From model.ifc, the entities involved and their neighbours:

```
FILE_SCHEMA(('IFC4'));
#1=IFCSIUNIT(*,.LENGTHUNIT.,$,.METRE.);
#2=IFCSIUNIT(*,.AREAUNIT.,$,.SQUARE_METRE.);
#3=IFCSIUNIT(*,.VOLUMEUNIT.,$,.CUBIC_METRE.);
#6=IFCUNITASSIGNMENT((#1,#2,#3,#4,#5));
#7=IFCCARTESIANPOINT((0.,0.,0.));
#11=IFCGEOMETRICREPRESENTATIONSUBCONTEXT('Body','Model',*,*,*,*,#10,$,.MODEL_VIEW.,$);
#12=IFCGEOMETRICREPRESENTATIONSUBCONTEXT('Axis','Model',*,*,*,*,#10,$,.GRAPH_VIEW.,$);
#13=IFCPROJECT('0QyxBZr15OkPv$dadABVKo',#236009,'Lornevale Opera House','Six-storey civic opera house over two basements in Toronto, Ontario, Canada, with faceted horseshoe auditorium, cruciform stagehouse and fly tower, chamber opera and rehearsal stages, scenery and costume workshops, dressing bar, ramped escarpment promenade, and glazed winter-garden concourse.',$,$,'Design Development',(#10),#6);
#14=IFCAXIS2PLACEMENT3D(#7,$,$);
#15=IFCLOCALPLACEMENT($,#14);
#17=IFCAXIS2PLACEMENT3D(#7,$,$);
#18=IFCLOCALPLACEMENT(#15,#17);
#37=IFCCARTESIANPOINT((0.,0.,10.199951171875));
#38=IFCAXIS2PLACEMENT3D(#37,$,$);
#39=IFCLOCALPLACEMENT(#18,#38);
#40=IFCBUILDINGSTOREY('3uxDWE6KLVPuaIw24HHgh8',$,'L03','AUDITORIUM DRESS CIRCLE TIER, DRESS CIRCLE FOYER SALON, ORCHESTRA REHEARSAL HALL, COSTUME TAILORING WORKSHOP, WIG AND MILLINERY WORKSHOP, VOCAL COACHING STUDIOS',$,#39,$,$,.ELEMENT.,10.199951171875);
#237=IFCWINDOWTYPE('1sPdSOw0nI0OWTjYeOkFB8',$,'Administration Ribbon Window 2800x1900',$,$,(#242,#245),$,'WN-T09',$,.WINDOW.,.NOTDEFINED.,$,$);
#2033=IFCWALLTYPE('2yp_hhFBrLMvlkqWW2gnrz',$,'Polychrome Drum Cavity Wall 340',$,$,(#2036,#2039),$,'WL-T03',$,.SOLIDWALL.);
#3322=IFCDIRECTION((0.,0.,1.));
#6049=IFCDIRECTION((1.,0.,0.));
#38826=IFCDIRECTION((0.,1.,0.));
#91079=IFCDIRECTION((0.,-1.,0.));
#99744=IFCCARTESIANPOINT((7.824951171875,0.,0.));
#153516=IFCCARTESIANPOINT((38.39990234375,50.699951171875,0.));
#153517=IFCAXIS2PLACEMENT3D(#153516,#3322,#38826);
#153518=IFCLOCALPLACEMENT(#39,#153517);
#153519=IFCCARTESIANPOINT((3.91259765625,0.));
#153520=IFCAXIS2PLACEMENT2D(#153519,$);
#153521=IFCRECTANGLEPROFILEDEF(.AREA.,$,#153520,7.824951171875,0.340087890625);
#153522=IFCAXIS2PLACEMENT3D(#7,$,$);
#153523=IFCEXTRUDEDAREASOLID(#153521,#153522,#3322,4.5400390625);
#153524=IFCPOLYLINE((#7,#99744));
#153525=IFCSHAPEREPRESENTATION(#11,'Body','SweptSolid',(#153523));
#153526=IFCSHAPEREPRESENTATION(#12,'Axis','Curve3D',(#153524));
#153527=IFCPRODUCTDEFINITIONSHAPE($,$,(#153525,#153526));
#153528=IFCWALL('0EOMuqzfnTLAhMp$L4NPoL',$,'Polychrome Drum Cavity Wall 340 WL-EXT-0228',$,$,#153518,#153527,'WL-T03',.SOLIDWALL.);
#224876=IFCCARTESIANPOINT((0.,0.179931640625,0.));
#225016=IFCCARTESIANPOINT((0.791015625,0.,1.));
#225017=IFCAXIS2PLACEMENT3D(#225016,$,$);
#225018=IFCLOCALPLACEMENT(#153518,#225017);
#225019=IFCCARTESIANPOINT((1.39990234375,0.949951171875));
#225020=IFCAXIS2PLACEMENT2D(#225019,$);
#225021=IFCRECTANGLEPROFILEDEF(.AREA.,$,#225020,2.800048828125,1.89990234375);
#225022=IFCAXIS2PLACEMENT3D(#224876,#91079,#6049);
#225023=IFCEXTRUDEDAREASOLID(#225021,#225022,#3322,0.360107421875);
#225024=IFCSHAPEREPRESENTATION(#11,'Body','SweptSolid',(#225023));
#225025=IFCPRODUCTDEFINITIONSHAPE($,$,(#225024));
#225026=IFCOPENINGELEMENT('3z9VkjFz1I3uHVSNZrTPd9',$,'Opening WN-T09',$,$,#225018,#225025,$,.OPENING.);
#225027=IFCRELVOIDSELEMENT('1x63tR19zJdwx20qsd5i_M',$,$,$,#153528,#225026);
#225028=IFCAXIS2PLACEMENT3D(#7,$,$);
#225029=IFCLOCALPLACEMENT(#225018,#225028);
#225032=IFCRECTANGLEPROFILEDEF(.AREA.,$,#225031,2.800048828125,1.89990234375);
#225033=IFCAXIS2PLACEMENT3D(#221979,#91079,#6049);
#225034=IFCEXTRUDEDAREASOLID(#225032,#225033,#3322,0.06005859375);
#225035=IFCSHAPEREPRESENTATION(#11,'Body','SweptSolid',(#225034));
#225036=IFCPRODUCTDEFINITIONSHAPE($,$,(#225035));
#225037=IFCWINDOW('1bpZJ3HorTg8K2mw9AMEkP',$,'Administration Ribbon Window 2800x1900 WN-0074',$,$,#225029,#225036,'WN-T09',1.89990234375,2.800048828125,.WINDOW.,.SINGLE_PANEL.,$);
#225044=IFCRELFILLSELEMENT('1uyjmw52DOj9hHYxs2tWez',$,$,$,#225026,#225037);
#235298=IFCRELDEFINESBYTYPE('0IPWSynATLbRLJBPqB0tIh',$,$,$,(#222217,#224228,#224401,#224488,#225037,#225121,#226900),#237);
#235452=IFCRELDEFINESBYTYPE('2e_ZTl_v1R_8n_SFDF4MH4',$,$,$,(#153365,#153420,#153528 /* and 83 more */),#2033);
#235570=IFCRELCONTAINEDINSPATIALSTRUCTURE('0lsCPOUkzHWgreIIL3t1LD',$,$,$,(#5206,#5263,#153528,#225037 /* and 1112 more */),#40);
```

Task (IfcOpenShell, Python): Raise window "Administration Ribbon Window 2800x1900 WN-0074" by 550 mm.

```python
import numpy as np
import ifcopenshell
import ifcopenshell.api.geometry
import ifcopenshell.util.placement
import ifcopenshell.util.unit

model = ifcopenshell.open("model.ifc")
unit_scale = ifcopenshell.util.unit.calculate_unit_scale(model)

window = model.by_guid("1bpZJ3HorTg8K2mw9AMEkP")
opening = window.FillsVoids[0].RelatingOpeningElement
dz = 0.55

shift = np.array([0.0, 0.0, dz])
# The window is placed relative to its opening, so it follows when the opening moves.
matrix = ifcopenshell.util.placement.get_local_placement(opening.ObjectPlacement)
matrix[:3, 3] += shift
ifcopenshell.api.geometry.edit_object_placement(
    model, product=opening, matrix=matrix, is_si=False, should_transform_children=True
)

print(f"moved by {dz * unit_scale:+.3f} m")

model.write("model_edited.ifc")
```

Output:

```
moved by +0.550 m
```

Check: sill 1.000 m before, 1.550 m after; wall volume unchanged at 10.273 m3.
